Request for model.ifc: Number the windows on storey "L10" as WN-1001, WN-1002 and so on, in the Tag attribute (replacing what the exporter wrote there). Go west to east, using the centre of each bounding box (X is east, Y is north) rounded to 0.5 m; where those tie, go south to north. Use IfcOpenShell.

First a look at what the model holds.

```python
import ifcopenshell
import ifcopenshell.util.element
import ifcopenshell.util.placement

model = ifcopenshell.open("model.ifc")
print(model.schema)
storey = next(s for s in model.by_type("IfcBuildingStorey") if s.Name == "L10")
windows = [e for e in ifcopenshell.util.element.get_decomposition(storey) if e.is_a("IfcWindow")]
for e in sorted(windows, key=lambda e: e.id()):
    origin = ifcopenshell.util.placement.get_local_placement(e.ObjectPlacement)[:3, 3]
    print(e.id(), e.Tag, e.Name, origin.round(2) + 0.0, sep=" | ")
```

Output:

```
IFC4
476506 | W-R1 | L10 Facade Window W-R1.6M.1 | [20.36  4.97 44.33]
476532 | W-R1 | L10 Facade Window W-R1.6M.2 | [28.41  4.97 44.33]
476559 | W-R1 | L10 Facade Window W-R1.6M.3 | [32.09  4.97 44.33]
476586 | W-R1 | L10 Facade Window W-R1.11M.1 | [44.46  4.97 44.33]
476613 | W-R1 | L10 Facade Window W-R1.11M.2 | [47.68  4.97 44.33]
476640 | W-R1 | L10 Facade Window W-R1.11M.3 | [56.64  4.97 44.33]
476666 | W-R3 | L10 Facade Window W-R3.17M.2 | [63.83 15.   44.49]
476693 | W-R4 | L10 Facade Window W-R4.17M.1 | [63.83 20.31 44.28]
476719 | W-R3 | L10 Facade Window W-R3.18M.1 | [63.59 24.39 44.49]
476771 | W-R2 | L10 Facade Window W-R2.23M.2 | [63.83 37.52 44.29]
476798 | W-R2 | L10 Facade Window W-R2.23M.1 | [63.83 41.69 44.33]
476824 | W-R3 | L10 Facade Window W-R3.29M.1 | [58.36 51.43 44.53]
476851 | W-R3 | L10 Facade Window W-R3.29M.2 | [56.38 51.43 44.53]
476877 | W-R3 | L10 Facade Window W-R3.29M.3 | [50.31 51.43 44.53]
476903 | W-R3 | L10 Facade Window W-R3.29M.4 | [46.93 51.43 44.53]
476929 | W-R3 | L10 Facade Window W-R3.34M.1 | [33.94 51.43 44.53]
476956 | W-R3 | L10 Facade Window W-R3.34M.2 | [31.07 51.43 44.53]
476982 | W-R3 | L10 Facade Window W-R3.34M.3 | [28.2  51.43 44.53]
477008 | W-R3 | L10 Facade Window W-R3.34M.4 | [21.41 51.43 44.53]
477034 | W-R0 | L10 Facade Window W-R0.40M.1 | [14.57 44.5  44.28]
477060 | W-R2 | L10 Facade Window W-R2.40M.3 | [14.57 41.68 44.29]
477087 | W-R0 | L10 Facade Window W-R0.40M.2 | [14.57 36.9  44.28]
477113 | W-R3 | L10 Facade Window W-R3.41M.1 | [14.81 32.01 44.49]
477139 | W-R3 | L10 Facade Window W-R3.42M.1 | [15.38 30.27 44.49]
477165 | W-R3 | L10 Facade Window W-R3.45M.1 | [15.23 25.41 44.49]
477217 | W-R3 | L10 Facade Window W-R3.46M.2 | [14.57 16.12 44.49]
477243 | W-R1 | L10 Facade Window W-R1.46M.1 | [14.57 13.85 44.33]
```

```python
import ifcopenshell
import ifcopenshell.geom
import ifcopenshell.util.element
import ifcopenshell.util.shape

model = ifcopenshell.open("model.ifc")
settings = ifcopenshell.geom.settings()
settings.set("use-world-coords", True)


def centre(element):
    shape = ifcopenshell.geom.create_shape(settings, element)
    return ifcopenshell.util.shape.get_bbox_centroid(shape.geometry)


storey = next(s for s in model.by_type("IfcBuildingStorey") if s.Name == "L10")
windows = [e for e in ifcopenshell.util.element.get_decomposition(storey) if e.is_a("IfcWindow")]

# Insertion points can sit at a corner or the storey origin, so sort by the geometry (in metres).
centres = {e: centre(e) for e in windows}
windows.sort(key=lambda e: (round(centres[e][0] / 0.5), centres[e][1]))

for i, e in enumerate(windows, start=1):
    number = f"WN-10{i:02d}"
    e.Tag = number
    print(e.id(), number)

model.write("model_rev.ifc")
```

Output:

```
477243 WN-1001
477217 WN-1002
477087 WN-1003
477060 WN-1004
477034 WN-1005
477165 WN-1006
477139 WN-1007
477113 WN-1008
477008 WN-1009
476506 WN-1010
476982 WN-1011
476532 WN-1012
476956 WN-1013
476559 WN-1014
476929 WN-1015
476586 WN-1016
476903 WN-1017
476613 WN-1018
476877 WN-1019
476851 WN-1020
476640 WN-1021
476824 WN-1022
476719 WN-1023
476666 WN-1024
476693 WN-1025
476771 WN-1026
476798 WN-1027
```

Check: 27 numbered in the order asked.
